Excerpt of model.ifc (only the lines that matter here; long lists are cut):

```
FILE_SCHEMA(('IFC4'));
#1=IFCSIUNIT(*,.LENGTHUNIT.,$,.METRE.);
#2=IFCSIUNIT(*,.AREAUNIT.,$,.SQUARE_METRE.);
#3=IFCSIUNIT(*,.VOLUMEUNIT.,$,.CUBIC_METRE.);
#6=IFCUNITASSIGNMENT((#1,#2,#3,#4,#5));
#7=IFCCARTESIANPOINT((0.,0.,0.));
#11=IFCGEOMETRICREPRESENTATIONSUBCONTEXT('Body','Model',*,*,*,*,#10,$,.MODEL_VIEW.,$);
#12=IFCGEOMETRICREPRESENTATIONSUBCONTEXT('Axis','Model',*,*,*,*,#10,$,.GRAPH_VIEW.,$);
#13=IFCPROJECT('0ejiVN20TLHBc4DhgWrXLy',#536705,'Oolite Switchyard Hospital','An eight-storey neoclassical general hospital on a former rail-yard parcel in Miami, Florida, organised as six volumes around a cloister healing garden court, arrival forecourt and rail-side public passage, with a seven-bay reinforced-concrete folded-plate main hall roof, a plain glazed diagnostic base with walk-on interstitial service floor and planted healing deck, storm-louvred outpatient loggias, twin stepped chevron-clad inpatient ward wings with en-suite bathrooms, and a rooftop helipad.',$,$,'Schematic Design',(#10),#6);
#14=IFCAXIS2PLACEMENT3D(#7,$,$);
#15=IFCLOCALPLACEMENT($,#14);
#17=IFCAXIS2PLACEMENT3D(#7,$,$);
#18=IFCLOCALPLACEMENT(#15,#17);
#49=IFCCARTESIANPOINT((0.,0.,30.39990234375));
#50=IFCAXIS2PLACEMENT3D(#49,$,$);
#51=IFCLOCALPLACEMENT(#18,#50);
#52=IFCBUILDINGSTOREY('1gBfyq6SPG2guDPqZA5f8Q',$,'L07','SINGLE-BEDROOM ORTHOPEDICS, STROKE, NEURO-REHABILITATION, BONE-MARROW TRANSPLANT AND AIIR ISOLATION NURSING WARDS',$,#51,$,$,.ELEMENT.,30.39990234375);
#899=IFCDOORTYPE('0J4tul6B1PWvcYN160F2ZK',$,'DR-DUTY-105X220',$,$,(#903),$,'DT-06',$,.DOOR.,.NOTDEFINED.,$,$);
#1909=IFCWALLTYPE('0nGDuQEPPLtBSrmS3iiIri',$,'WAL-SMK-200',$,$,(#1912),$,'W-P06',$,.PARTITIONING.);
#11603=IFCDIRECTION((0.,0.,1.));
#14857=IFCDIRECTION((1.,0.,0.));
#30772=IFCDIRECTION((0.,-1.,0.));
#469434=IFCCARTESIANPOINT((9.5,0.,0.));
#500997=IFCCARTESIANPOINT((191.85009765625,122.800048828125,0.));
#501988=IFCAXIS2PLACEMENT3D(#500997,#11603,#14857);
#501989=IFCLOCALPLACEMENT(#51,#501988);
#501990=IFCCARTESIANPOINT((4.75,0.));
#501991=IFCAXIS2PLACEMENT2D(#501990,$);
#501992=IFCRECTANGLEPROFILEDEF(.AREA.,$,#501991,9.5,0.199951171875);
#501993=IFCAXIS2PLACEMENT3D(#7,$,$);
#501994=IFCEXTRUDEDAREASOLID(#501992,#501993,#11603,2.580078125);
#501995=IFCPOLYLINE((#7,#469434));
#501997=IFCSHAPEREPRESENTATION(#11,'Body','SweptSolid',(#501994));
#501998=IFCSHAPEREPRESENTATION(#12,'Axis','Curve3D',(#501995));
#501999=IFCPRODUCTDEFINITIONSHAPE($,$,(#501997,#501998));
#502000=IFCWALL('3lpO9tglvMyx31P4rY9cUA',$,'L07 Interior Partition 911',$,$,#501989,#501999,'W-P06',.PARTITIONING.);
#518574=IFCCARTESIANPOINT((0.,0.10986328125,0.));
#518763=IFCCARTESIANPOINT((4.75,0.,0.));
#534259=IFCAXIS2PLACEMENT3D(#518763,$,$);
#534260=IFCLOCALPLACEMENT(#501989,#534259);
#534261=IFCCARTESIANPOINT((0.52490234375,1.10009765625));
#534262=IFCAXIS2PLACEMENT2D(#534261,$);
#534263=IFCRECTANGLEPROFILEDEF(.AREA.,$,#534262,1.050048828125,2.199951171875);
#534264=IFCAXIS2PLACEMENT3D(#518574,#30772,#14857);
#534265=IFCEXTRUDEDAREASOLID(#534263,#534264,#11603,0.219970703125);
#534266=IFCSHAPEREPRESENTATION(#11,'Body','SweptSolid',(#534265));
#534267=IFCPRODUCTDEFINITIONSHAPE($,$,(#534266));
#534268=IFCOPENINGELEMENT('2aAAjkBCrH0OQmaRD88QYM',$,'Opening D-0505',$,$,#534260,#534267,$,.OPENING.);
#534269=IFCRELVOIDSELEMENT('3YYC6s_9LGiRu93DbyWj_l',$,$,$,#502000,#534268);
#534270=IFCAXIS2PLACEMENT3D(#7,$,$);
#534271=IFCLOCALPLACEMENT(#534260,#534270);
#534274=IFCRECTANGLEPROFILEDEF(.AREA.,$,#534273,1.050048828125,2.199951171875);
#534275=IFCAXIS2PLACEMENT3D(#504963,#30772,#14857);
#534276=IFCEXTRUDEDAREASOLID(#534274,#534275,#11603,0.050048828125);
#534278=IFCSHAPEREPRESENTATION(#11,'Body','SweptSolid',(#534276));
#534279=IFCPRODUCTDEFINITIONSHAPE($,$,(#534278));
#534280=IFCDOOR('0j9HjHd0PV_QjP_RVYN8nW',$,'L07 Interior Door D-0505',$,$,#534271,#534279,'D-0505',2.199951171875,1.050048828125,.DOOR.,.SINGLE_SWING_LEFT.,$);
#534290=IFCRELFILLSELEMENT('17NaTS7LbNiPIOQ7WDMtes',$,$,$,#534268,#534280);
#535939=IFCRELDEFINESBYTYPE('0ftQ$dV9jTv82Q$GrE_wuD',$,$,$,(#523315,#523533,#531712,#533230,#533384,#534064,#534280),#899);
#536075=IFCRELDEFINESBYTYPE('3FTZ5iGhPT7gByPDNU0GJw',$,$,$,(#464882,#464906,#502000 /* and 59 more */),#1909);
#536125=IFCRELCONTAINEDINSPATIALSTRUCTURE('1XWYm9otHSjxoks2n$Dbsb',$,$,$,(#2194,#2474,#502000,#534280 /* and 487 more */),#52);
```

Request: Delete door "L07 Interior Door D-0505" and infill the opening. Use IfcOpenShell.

```python
import ifcopenshell
import ifcopenshell.api.feature
import ifcopenshell.api.root
import ifcopenshell.geom
import ifcopenshell.util.shape

model = ifcopenshell.open("model.ifc")
settings = ifcopenshell.geom.settings()


def volume(element):
    """Net volume in cubic metres, openings subtracted."""
    shape = ifcopenshell.geom.create_shape(settings, element)
    return ifcopenshell.util.shape.get_volume(shape.geometry)


door = model.by_guid("0j9HjHd0PV_QjP_RVYN8nW")
opening = door.FillsVoids[0].RelatingOpeningElement
wall = opening.VoidsElements[0].RelatingBuildingElement
before = volume(wall)

ifcopenshell.api.root.remove_product(model, product=door)
ifcopenshell.api.feature.remove_feature(model, feature=opening)

after = volume(wall)

print(f"wall volume {before:.3f} -> {after:.3f} m3")

model.write("model_edited.ifc")
```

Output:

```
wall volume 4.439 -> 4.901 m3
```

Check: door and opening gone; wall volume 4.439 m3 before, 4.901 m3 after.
